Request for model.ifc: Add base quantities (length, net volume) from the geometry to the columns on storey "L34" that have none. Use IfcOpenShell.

First a look at what the model holds.

```python
import ifcopenshell
import ifcopenshell.util.element
import ifcopenshell.util.unit

model = ifcopenshell.open("model.ifc")
print(model.schema)
for unit_type in ("LENGTHUNIT", "AREAUNIT", "VOLUMEUNIT"):
    print(unit_type, ifcopenshell.util.unit.calculate_unit_scale(model, unit_type))
storey = next(s for s in model.by_type("IfcBuildingStorey") if s.Name == "L34")
columns = [e for e in ifcopenshell.util.element.get_decomposition(storey) if e.is_a("IfcColumn")]
for e in sorted(columns, key=lambda e: e.id()):
    print(e.id(), e.is_a(), e.Name, list(ifcopenshell.util.element.get_psets(e, qtos_only=True)), sep=" | ")
```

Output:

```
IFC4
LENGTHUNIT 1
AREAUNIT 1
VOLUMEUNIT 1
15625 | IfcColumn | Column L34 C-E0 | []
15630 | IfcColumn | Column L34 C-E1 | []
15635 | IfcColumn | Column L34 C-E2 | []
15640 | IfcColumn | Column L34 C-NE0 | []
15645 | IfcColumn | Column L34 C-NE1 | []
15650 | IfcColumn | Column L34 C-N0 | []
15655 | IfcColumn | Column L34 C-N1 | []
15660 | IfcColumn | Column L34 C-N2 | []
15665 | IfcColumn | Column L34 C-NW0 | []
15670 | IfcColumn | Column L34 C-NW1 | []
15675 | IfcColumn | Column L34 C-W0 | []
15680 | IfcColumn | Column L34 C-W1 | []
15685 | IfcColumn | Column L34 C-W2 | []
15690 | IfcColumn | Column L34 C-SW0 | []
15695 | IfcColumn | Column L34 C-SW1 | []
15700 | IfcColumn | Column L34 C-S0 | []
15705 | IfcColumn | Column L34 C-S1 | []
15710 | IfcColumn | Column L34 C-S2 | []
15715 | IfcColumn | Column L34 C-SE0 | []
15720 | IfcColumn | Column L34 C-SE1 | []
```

```python
import ifcopenshell
import ifcopenshell.api.pset
import ifcopenshell.geom
import ifcopenshell.util.element
import ifcopenshell.util.shape
import ifcopenshell.util.unit

model = ifcopenshell.open("model.ifc")
unit_scale = ifcopenshell.util.unit.calculate_unit_scale(model)
volume_scale = ifcopenshell.util.unit.calculate_unit_scale(model, "VOLUMEUNIT")
settings = ifcopenshell.geom.settings()

storey = next(s for s in model.by_type("IfcBuildingStorey") if s.Name == "L34")
columns = [e for e in ifcopenshell.util.element.get_decomposition(storey) if e.is_a("IfcColumn")]

for e in sorted(columns, key=lambda e: e.id()):
    if ifcopenshell.util.element.get_psets(e, qtos_only=True, should_inherit=False):
        continue
    # Geometry comes back in metres, in the element's own axes.
    shape = ifcopenshell.geom.create_shape(settings, e)
    values = {
        "Length": ifcopenshell.util.shape.get_z(shape.geometry) / unit_scale,
        "NetVolume": ifcopenshell.util.shape.get_volume(shape.geometry) / volume_scale,
    }
    qto = ifcopenshell.api.pset.add_qto(model, product=e, name="Qto_ColumnBaseQuantities")
    ifcopenshell.api.pset.edit_qto(model, qto=qto, properties=values)
    print(e.id(), {k: round(v, 3) for k, v in values.items()})

model.write("model_v2.ifc")
```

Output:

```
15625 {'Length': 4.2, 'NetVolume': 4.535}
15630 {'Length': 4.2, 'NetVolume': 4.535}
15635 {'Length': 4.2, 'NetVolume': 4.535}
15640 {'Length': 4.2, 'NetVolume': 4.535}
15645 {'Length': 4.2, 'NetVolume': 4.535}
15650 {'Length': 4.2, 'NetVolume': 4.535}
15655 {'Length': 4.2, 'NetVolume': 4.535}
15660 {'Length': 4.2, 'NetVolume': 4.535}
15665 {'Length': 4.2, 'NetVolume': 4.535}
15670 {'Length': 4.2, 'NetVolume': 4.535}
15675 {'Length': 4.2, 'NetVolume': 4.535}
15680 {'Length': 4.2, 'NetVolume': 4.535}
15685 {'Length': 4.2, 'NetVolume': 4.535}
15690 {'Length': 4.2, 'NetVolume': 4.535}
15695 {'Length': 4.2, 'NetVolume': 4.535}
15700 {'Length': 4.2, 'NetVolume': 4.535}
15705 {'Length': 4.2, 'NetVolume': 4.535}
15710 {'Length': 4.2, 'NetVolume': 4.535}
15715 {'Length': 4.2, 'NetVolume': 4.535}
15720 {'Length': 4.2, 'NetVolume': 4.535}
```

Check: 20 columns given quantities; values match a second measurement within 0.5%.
